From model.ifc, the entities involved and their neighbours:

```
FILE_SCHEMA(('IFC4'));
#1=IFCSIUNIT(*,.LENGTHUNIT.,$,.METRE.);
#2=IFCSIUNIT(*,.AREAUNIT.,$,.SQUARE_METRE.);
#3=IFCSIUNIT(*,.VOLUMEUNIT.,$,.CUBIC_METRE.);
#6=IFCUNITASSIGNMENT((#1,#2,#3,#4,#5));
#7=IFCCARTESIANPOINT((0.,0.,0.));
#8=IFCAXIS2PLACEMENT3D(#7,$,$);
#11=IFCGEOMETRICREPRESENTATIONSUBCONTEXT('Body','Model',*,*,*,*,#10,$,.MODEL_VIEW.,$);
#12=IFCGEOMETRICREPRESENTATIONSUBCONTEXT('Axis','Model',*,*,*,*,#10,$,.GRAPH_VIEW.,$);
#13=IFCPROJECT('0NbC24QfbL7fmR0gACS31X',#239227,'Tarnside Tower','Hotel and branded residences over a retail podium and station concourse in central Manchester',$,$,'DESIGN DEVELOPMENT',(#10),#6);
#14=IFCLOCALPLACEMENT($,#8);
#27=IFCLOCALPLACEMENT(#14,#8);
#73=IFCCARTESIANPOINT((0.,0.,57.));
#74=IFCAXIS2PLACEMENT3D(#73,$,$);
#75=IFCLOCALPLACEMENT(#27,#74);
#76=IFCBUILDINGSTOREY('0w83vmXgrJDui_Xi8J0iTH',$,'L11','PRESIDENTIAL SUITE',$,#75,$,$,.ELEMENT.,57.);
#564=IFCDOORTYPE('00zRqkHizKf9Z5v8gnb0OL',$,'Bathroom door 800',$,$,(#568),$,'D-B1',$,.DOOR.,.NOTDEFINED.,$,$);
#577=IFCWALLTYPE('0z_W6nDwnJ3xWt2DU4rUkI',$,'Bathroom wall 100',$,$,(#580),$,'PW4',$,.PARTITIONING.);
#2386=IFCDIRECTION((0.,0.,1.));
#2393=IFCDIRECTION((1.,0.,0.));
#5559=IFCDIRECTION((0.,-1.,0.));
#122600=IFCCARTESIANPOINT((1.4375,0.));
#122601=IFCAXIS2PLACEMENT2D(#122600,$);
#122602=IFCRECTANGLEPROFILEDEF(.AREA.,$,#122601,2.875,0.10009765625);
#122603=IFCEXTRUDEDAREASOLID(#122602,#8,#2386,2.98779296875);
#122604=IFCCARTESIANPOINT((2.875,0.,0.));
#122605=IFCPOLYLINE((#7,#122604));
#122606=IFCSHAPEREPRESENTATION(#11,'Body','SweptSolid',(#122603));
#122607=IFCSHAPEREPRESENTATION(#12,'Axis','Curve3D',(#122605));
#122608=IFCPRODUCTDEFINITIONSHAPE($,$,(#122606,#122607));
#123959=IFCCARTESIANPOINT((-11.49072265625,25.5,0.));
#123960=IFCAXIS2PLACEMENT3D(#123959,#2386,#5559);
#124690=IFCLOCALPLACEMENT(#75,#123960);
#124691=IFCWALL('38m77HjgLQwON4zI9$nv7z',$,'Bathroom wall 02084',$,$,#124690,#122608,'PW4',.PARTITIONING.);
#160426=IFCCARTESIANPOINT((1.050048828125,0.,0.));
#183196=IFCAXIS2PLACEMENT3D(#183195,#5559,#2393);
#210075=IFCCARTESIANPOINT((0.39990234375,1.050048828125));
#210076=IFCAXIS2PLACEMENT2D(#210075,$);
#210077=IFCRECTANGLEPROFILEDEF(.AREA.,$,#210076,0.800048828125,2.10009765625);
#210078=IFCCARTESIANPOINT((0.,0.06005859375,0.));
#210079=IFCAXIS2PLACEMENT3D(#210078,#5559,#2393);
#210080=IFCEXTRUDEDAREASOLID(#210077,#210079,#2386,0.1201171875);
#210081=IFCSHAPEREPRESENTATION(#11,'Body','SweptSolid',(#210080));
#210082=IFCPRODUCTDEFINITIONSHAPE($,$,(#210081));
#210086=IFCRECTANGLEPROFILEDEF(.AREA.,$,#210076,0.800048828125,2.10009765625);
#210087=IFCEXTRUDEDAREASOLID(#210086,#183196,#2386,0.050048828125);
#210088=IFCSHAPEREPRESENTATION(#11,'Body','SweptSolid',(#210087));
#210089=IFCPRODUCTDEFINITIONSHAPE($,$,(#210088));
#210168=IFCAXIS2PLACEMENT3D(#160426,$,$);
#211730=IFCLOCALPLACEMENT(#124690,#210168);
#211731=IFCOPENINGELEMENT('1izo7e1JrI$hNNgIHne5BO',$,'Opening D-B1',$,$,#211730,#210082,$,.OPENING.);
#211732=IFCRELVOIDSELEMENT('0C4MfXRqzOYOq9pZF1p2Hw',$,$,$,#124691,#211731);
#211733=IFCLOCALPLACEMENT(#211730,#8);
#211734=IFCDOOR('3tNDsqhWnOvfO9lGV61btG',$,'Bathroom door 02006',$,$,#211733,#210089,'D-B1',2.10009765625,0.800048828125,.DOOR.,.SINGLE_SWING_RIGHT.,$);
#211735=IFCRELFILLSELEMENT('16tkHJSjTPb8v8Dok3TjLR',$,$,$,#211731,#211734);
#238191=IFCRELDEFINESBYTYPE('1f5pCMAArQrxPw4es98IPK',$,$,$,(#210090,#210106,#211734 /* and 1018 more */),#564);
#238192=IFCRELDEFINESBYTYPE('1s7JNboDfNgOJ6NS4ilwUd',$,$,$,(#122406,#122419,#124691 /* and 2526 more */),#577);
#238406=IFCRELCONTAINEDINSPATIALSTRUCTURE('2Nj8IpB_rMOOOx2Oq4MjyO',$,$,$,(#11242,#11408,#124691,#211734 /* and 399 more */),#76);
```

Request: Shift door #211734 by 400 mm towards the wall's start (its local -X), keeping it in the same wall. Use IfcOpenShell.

```python
import ifcopenshell
import ifcopenshell.api.geometry
import ifcopenshell.util.placement
import ifcopenshell.util.unit

model = ifcopenshell.open("model.ifc")
unit_scale = ifcopenshell.util.unit.calculate_unit_scale(model)

door = model.by_guid("3tNDsqhWnOvfO9lGV61btG")
opening = door.FillsVoids[0].RelatingOpeningElement
wall = opening.VoidsElements[0].RelatingBuildingElement

wall_matrix = ifcopenshell.util.placement.get_local_placement(wall.ObjectPlacement)
shift = wall_matrix[:3, 0] * -0.4 / unit_scale
before = ifcopenshell.util.placement.get_local_placement(door.ObjectPlacement)[:3, 3].copy()

# The door is placed relative to its opening, so it follows when the opening moves.
matrix = ifcopenshell.util.placement.get_local_placement(opening.ObjectPlacement)
matrix[:3, 3] += shift
ifcopenshell.api.geometry.edit_object_placement(
    model, product=opening, matrix=matrix, is_si=False, should_transform_children=True
)

after = ifcopenshell.util.placement.get_local_placement(door.ObjectPlacement)[:3, 3]
print("door moved by", (after - before).round(3) + 0.0)

model.write("model_rev.ifc")
```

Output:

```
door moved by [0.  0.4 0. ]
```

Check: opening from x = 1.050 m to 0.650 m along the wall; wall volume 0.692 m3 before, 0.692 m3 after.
